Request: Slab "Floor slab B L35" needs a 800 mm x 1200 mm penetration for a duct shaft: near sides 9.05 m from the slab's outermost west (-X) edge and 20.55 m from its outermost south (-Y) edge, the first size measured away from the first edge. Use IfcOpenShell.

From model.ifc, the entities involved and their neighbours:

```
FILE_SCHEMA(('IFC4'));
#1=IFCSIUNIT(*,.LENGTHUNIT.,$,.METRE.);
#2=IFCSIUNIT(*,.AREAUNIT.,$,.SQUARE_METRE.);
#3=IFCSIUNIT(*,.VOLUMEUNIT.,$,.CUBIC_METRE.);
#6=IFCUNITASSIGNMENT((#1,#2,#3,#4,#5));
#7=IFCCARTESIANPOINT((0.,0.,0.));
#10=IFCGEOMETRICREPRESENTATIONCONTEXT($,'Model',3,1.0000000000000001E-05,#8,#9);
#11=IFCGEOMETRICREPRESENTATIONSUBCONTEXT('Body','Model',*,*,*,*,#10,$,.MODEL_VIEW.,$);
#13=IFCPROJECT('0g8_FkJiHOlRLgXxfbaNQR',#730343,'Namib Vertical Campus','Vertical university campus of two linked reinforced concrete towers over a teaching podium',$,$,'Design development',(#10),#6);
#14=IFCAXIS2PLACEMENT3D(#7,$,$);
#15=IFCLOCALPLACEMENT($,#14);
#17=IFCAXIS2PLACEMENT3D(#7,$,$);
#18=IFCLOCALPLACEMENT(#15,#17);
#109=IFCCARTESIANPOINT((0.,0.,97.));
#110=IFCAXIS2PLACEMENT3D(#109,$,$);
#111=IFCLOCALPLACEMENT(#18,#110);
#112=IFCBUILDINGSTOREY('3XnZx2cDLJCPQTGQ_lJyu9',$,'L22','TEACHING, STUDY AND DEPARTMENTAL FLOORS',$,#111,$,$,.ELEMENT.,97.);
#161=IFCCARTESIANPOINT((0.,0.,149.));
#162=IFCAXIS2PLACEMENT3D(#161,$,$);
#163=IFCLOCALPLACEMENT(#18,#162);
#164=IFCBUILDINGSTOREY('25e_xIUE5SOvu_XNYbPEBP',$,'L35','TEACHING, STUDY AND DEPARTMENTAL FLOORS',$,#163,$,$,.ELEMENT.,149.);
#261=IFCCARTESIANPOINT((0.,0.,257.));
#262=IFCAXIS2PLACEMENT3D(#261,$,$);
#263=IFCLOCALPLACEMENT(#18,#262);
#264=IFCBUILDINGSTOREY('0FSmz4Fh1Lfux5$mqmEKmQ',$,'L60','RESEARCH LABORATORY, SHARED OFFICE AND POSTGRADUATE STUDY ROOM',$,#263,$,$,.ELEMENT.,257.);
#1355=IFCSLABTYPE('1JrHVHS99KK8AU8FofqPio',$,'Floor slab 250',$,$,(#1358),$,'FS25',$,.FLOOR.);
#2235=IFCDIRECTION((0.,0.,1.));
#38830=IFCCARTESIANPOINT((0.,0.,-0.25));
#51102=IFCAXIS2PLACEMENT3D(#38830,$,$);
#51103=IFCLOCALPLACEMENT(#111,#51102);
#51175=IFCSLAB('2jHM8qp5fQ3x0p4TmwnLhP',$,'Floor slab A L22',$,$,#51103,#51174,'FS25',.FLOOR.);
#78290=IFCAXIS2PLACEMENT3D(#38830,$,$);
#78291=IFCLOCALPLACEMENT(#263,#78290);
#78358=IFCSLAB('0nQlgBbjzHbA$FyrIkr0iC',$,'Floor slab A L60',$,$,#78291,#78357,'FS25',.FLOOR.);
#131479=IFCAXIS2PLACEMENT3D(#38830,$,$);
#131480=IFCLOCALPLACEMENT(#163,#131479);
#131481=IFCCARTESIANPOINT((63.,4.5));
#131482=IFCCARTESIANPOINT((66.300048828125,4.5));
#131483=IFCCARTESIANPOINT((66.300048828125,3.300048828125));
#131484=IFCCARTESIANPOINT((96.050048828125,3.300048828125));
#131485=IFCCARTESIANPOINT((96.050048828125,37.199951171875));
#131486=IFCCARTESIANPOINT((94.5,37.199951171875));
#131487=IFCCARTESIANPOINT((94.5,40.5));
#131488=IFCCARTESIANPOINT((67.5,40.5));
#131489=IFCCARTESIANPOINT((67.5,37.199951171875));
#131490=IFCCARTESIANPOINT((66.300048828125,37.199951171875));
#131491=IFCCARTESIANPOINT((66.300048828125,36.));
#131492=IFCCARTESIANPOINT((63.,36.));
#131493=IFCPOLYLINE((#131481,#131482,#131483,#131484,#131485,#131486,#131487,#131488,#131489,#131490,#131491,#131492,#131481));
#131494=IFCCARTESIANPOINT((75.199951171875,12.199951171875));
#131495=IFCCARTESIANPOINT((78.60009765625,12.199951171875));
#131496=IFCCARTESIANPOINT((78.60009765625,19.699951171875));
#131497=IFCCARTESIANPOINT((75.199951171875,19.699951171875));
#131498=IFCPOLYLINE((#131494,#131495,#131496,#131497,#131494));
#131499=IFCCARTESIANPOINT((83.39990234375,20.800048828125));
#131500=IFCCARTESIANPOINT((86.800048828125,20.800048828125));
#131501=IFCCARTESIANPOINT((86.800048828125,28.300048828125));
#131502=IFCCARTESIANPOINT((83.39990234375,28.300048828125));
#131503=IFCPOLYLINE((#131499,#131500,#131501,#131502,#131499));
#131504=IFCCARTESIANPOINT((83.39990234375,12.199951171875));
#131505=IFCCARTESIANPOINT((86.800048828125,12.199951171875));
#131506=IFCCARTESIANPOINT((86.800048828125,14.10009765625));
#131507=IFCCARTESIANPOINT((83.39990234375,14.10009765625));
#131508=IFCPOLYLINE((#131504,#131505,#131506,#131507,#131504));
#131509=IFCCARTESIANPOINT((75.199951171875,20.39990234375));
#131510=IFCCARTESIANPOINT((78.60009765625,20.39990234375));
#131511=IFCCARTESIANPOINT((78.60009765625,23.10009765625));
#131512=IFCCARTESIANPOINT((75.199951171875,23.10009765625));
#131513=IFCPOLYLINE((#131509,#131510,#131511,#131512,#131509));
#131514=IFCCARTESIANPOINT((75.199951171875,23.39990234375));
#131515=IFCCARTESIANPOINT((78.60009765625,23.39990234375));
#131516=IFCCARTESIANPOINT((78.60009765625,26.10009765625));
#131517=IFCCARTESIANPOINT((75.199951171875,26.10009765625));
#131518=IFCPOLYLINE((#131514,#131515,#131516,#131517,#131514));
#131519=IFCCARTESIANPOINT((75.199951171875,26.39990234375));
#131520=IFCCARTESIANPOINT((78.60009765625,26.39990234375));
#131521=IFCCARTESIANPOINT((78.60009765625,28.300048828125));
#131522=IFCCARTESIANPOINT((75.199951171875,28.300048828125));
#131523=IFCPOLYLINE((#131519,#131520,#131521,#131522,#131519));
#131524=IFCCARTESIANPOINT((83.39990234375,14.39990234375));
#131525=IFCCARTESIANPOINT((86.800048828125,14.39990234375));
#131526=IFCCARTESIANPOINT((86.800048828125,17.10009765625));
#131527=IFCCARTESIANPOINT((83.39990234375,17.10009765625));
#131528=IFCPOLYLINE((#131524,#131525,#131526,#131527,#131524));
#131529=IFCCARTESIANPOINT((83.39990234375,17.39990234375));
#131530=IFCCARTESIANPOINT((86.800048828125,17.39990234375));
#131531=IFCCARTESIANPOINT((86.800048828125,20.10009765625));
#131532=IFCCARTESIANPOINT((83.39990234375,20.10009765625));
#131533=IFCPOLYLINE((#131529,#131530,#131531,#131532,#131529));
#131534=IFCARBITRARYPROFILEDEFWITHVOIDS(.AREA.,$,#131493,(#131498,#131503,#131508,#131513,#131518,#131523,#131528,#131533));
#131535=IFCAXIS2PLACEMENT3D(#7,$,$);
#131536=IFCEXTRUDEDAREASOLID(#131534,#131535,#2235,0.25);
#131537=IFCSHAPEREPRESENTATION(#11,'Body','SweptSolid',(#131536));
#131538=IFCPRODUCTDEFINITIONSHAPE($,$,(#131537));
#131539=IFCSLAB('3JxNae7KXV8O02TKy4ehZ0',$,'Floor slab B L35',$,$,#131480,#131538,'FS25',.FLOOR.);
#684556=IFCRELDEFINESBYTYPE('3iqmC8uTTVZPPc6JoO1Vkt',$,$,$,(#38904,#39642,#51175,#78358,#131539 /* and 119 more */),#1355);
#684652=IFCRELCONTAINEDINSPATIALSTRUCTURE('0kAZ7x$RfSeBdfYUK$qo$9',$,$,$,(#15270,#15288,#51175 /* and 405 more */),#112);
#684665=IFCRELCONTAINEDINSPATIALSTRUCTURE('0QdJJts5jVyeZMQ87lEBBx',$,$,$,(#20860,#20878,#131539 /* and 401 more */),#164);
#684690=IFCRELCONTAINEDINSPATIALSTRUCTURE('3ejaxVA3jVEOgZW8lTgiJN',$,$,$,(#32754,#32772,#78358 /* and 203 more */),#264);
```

```python
import numpy as np
import ifcopenshell
import ifcopenshell.api.feature
import ifcopenshell.api.geometry
import ifcopenshell.api.root
import ifcopenshell.geom
import ifcopenshell.util.placement
import ifcopenshell.util.representation
import ifcopenshell.util.shape
import ifcopenshell.util.unit

model = ifcopenshell.open("model.ifc")
unit_scale = ifcopenshell.util.unit.calculate_unit_scale(model)
settings = ifcopenshell.geom.settings()


def volume(element):
    """Net volume in cubic metres, openings subtracted."""
    shape = ifcopenshell.geom.create_shape(settings, element)
    return ifcopenshell.util.shape.get_volume(shape.geometry)


slab = model.by_guid("3JxNae7KXV8O02TKy4ehZ0")
before = volume(slab)

# Extent in the slab's own axes, in metres. The edges named are its -X and -Y sides.
slab_shape = ifcopenshell.geom.create_shape(settings, slab)
vertices = ifcopenshell.util.shape.get_vertices(slab_shape.geometry)
x_min, y_min, bottom = vertices.min(axis=0)
top = vertices[:, 2].max()

opening = ifcopenshell.api.root.create_entity(model, ifc_class="IfcOpeningElement", name="Duct shaft opening", predefined_type="OPENING")
context = ifcopenshell.util.representation.get_context(model, "Model", "Body", "MODEL_VIEW")
width, depth = 0.8, 1.2
outline = [(0.0, 0.0), (width, 0.0), (width, depth), (0.0, depth), (0.0, 0.0)]
# Overshoot both faces by 50 mm so the cut is clean.
shape = ifcopenshell.api.geometry.add_slab_representation(
    model, context=context, depth=top - bottom + 0.1, polyline=outline
)
ifcopenshell.api.geometry.assign_representation(model, product=opening, representation=shape)

matrix = ifcopenshell.util.placement.get_local_placement(slab.ObjectPlacement)
matrix[:, 3] = matrix @ np.append(np.array([x_min + 9.05, y_min + 20.55, bottom - 0.05]) / unit_scale, 1.0)
ifcopenshell.api.geometry.edit_object_placement(model, product=opening, matrix=matrix, is_si=False)
ifcopenshell.api.feature.add_feature(model, feature=opening, element=slab)

after = volume(slab)

print(f"slab volume {before:.3f} -> {after:.3f} m3")

model.write("model_rev.ifc")
```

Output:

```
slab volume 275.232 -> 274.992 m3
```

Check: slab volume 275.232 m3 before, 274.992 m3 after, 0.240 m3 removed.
